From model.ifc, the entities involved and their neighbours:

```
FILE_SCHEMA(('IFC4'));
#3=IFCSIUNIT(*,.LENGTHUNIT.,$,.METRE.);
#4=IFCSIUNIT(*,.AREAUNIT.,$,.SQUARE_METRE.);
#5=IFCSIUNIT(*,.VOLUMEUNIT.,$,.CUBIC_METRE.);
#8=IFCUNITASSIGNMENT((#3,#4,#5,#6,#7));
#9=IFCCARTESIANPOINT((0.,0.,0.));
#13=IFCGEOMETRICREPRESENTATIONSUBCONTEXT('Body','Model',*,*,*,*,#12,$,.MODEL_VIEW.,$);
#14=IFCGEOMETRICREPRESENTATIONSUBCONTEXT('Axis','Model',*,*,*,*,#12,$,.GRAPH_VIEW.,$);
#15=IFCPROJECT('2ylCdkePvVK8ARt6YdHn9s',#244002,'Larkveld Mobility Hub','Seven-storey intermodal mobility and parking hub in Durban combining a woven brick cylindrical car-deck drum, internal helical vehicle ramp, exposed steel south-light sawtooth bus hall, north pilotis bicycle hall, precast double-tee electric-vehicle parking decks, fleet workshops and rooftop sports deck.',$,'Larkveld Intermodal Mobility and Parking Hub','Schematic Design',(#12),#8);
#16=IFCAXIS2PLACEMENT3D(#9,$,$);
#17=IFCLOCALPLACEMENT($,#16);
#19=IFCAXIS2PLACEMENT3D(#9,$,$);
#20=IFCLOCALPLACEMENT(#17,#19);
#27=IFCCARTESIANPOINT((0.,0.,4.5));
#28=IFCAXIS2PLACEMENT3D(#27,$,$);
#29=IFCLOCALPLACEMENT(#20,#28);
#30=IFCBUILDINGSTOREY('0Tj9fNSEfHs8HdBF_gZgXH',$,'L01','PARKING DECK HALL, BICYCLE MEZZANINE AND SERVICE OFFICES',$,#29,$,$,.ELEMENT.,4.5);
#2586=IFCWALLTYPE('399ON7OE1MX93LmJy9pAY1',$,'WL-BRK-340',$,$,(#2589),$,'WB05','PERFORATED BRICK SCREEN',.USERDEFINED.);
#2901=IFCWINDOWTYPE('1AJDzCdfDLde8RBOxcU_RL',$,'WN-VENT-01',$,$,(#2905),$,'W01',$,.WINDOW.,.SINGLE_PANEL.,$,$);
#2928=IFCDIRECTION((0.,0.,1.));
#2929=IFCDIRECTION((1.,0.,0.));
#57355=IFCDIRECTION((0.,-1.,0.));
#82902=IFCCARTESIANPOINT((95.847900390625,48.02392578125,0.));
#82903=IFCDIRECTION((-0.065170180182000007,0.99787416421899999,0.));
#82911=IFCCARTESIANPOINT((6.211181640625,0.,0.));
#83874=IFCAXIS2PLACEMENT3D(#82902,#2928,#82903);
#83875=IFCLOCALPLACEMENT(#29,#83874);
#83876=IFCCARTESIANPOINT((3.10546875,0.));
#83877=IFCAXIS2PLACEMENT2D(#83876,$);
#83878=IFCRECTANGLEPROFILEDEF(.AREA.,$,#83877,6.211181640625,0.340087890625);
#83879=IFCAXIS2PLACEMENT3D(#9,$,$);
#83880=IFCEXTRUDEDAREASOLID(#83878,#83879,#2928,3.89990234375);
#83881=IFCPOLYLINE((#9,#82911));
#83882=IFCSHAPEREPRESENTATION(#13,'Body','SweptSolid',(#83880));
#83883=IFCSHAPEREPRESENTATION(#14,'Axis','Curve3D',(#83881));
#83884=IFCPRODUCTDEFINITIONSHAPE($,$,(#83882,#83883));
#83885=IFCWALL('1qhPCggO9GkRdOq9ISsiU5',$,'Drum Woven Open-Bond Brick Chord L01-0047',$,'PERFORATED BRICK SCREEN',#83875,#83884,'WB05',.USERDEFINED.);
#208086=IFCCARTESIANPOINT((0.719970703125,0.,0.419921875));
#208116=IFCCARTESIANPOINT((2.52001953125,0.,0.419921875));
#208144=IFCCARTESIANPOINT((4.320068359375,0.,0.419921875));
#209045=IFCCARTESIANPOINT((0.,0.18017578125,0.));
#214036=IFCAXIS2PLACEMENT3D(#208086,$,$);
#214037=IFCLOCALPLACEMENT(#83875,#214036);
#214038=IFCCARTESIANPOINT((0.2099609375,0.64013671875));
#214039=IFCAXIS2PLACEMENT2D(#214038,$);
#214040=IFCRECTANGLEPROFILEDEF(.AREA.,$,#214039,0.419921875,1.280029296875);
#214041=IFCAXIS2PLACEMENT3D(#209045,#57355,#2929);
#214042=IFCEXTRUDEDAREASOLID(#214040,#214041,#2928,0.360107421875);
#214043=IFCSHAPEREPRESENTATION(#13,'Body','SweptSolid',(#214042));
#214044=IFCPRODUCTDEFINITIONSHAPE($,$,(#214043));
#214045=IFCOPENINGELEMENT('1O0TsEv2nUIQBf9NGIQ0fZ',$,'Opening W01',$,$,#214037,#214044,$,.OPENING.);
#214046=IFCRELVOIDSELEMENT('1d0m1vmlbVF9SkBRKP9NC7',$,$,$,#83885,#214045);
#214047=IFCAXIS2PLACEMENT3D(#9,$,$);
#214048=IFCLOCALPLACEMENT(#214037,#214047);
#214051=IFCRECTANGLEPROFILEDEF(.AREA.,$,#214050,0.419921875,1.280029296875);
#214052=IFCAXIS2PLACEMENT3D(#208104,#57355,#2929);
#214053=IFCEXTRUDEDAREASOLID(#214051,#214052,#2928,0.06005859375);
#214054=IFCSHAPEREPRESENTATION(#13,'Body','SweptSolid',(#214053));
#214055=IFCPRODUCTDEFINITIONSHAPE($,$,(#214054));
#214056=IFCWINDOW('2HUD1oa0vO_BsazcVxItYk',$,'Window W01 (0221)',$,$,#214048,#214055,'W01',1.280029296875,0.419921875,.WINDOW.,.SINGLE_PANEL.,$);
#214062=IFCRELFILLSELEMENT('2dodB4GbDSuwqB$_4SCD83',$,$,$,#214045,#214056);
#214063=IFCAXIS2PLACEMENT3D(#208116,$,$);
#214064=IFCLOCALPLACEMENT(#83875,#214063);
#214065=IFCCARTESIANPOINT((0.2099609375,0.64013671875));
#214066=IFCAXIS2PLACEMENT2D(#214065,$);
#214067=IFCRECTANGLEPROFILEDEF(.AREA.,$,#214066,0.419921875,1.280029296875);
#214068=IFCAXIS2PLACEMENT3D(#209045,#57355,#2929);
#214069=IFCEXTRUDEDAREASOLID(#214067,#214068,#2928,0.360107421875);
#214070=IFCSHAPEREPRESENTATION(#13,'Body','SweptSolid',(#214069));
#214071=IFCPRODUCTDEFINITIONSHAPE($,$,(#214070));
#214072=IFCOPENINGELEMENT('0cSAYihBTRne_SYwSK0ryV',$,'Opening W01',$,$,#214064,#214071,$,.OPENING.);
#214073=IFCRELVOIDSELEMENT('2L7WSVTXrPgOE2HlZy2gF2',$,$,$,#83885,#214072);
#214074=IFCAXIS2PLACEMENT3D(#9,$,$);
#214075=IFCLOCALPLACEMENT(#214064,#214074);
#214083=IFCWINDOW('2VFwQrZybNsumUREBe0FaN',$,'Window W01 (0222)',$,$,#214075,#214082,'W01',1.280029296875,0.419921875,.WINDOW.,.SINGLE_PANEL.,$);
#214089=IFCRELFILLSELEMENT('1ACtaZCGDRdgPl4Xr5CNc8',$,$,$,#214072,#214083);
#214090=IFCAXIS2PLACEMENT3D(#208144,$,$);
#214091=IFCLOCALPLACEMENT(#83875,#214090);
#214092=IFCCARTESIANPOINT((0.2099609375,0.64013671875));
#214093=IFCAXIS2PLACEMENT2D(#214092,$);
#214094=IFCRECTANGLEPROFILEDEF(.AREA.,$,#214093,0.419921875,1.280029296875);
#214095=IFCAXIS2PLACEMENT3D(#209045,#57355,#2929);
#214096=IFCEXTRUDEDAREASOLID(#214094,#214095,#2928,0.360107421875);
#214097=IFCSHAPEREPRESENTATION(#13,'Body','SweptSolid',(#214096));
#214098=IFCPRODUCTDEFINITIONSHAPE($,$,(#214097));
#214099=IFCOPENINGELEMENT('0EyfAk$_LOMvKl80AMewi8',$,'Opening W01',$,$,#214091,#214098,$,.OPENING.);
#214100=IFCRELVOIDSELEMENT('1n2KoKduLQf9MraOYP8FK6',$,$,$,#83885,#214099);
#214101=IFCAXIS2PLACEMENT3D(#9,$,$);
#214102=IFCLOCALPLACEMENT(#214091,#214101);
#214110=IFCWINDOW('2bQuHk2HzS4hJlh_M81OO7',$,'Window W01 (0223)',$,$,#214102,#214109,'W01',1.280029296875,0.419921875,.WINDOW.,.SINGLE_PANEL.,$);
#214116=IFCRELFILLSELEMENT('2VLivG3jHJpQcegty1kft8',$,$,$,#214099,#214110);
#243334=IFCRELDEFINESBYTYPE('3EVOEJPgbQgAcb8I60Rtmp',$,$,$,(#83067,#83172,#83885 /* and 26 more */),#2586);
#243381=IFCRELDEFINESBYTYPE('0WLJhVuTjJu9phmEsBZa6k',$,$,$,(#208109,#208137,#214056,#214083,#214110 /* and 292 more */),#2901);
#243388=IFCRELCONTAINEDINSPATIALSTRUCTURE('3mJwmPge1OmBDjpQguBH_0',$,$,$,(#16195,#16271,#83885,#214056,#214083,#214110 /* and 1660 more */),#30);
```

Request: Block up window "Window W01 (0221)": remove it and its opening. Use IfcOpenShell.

```python
import ifcopenshell
import ifcopenshell.api.feature
import ifcopenshell.api.root
import ifcopenshell.geom
import ifcopenshell.util.shape

model = ifcopenshell.open("model.ifc")
settings = ifcopenshell.geom.settings()


def volume(element):
    """Net volume in cubic metres, openings subtracted."""
    shape = ifcopenshell.geom.create_shape(settings, element)
    return ifcopenshell.util.shape.get_volume(shape.geometry)


window = model.by_guid("2HUD1oa0vO_BsazcVxItYk")
opening = window.FillsVoids[0].RelatingOpeningElement
wall = opening.VoidsElements[0].RelatingBuildingElement
before = volume(wall)

ifcopenshell.api.root.remove_product(model, product=window)
ifcopenshell.api.feature.remove_feature(model, feature=opening)

after = volume(wall)

print(f"wall volume {before:.3f} -> {after:.3f} m3")

model.write("model_edited.ifc")
```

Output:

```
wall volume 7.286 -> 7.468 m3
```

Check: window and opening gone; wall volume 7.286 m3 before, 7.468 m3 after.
